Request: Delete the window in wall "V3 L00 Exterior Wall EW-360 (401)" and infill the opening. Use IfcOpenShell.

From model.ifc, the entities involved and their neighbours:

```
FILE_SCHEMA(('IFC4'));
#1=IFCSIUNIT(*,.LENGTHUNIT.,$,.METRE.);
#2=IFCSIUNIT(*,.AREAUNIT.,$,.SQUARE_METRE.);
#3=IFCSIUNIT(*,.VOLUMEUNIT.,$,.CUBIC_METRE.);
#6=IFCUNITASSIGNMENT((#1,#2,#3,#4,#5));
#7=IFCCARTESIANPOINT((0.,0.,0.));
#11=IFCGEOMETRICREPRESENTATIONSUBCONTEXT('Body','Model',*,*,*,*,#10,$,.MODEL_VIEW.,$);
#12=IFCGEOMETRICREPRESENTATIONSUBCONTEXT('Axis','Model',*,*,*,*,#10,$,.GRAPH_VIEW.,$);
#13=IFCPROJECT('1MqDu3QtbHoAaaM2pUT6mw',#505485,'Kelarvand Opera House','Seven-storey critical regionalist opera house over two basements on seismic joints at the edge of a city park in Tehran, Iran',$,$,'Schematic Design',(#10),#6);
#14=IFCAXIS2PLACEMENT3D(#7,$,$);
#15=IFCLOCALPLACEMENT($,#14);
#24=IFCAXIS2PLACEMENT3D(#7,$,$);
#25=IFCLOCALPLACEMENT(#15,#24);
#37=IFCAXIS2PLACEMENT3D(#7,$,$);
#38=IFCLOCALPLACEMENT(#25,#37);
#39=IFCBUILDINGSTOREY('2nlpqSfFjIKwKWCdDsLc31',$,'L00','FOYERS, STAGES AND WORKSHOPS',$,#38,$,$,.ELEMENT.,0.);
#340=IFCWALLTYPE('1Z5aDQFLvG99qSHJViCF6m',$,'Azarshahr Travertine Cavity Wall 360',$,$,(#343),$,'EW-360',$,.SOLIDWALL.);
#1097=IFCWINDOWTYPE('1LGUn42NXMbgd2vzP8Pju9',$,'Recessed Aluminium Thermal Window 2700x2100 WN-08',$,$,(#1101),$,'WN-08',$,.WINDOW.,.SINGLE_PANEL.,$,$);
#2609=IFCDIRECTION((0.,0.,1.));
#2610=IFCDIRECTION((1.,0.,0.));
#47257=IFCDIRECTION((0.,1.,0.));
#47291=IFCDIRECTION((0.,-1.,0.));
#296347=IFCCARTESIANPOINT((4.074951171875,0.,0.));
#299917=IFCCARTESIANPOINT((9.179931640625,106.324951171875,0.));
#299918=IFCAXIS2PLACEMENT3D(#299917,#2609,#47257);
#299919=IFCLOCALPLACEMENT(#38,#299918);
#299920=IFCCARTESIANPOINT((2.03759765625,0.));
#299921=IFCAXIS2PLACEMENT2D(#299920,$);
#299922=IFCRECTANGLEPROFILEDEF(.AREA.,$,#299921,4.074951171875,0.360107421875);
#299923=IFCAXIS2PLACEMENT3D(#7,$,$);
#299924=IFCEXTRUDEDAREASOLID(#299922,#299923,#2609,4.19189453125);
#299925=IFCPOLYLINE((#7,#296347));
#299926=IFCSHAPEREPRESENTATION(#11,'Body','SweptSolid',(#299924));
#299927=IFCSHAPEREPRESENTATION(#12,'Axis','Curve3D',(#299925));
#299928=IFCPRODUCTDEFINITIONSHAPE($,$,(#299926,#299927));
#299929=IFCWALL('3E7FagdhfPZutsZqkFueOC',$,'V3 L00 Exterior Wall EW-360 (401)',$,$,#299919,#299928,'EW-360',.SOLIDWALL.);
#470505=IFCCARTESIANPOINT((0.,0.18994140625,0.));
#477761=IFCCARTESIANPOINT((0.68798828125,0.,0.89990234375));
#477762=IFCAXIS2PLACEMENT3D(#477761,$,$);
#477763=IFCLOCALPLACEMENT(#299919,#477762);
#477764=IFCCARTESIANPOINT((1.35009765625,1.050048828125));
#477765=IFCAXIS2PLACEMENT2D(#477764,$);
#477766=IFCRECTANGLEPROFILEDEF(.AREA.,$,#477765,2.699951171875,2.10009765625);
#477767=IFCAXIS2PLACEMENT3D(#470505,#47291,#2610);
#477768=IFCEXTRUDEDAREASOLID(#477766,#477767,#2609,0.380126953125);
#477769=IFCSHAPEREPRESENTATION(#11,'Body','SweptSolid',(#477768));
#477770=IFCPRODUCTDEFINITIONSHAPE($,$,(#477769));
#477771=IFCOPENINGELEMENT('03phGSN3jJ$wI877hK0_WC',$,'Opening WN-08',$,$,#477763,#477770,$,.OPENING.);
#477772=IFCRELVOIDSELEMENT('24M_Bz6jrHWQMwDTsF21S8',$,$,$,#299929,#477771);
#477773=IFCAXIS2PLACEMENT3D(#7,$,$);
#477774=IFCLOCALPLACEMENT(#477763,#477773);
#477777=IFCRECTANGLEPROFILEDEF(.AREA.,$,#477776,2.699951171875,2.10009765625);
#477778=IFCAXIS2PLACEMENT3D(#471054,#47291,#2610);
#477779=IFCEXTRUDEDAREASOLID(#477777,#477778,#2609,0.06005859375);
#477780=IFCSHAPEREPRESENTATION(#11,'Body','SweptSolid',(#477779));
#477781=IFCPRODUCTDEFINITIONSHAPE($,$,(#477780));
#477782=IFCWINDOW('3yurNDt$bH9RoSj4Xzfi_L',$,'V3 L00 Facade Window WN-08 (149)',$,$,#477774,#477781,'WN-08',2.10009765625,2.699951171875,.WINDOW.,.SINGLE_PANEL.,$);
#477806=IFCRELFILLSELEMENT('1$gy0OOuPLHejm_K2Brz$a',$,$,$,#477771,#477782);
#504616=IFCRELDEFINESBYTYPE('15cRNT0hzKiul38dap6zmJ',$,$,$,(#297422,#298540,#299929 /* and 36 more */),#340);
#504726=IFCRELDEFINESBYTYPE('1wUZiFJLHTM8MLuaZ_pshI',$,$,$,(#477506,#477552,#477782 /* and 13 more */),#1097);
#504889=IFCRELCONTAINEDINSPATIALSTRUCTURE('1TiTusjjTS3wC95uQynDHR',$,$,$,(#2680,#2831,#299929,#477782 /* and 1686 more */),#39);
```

```python
import ifcopenshell
import ifcopenshell.api.feature
import ifcopenshell.api.root
import ifcopenshell.geom
import ifcopenshell.util.shape

model = ifcopenshell.open("model.ifc")
settings = ifcopenshell.geom.settings()


def volume(element):
    """Net volume in cubic metres, openings subtracted."""
    shape = ifcopenshell.geom.create_shape(settings, element)
    return ifcopenshell.util.shape.get_volume(shape.geometry)


window = model.by_guid("3yurNDt$bH9RoSj4Xzfi_L")
opening = window.FillsVoids[0].RelatingOpeningElement
wall = opening.VoidsElements[0].RelatingBuildingElement
before = volume(wall)

ifcopenshell.api.root.remove_product(model, product=window)
ifcopenshell.api.feature.remove_feature(model, feature=opening)

after = volume(wall)

print(f"wall volume {before:.3f} -> {after:.3f} m3")

model.write("model_rev.ifc")
```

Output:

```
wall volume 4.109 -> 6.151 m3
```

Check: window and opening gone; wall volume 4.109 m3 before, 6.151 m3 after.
